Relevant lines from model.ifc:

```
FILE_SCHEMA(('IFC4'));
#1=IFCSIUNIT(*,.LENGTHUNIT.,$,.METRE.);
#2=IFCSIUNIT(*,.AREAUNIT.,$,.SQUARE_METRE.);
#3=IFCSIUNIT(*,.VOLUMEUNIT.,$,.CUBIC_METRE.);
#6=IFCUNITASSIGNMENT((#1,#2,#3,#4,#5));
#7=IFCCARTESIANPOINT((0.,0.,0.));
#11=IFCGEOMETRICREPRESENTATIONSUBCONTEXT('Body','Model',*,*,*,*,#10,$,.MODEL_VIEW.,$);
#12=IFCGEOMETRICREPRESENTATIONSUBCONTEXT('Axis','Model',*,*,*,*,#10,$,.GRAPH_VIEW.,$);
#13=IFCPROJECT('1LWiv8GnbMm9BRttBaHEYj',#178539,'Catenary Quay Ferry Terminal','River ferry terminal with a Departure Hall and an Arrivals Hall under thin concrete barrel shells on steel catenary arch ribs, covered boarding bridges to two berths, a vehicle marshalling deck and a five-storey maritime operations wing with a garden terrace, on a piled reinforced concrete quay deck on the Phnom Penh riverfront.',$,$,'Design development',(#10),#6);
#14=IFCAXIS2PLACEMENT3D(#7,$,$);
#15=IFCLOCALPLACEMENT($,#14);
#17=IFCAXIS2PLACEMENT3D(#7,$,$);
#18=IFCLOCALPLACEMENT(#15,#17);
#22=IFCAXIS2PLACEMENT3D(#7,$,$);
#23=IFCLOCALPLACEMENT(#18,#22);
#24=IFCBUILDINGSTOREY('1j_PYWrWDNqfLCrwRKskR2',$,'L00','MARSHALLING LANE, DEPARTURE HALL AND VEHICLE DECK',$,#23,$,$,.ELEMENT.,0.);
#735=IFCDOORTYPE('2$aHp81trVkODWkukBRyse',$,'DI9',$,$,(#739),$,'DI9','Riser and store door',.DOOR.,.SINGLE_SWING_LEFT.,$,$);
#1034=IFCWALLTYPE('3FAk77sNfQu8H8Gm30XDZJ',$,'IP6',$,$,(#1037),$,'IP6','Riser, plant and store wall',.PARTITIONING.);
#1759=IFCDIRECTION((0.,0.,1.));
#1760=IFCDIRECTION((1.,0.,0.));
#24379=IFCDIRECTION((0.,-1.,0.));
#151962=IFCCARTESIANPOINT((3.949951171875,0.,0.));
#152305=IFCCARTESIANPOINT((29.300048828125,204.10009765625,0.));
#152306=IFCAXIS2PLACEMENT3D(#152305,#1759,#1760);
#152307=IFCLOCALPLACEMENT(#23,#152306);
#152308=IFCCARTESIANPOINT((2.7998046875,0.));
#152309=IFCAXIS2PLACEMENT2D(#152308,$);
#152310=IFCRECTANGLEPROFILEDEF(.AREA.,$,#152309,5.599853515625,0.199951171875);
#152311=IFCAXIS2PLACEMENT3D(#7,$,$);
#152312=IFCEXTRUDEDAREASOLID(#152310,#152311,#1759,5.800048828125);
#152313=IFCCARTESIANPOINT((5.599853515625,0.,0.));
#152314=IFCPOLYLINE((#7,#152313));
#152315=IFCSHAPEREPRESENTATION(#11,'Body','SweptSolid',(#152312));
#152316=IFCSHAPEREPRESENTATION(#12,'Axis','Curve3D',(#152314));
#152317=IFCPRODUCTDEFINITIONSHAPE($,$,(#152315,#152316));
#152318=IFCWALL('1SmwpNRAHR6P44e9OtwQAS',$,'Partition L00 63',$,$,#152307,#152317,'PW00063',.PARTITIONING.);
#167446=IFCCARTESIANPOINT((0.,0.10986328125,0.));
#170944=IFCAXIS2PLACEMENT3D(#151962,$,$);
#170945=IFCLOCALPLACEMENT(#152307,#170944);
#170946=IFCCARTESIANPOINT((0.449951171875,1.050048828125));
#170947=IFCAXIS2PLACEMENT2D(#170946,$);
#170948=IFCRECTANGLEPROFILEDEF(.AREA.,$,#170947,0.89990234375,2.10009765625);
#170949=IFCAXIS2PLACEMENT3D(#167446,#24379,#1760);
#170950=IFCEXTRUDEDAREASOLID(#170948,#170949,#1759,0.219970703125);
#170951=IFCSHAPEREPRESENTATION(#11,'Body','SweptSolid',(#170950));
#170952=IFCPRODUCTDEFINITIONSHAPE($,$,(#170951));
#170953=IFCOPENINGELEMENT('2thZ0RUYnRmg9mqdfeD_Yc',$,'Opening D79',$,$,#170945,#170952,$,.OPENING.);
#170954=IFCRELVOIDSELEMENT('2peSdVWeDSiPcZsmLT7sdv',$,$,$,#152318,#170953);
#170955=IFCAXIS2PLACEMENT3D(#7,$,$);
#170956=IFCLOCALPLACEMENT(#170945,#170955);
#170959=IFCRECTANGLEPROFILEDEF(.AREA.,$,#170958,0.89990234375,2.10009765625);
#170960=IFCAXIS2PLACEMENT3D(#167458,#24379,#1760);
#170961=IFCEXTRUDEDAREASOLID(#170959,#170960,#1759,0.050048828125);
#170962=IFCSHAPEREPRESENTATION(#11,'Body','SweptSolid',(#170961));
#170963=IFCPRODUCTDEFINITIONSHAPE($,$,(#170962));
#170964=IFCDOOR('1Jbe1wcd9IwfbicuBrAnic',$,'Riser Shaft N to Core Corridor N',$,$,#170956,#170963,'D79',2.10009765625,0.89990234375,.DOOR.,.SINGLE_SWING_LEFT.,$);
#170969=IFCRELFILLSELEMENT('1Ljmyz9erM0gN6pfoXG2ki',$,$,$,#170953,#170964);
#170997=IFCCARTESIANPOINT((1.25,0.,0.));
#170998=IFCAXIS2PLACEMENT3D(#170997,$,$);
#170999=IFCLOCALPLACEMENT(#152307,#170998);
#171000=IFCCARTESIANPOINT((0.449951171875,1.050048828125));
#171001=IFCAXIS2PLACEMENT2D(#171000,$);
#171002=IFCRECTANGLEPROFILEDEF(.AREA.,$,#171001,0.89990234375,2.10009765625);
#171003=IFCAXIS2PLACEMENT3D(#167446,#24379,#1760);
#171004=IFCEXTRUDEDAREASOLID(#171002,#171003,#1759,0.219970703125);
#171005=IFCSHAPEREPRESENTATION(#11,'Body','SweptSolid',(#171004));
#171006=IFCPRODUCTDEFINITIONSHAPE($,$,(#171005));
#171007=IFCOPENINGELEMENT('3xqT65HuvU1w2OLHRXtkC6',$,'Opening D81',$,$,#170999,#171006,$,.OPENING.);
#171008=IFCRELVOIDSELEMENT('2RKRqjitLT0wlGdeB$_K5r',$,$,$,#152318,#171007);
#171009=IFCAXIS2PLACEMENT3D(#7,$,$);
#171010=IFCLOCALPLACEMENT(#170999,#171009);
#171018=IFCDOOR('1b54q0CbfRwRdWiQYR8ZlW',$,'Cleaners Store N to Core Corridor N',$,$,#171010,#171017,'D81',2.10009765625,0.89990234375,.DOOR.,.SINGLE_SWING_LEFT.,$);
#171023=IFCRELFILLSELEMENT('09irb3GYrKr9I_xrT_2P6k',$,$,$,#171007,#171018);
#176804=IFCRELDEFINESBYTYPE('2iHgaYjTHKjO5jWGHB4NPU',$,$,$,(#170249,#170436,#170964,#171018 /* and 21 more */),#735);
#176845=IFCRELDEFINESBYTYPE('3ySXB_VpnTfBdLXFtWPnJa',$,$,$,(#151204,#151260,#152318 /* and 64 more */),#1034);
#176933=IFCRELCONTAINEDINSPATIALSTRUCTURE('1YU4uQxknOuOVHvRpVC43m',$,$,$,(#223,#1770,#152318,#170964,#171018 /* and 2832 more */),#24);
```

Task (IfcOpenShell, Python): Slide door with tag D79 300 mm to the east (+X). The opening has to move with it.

```python
import ifcopenshell
import ifcopenshell.api.geometry
import ifcopenshell.util.placement
import ifcopenshell.util.unit

model = ifcopenshell.open("model.ifc")
unit_scale = ifcopenshell.util.unit.calculate_unit_scale(model)

door = model.by_guid("1Jbe1wcd9IwfbicuBrAnic")
opening = door.FillsVoids[0].RelatingOpeningElement
wall = opening.VoidsElements[0].RelatingBuildingElement

wall_matrix = ifcopenshell.util.placement.get_local_placement(wall.ObjectPlacement)
shift = wall_matrix[:3, 0] * 0.3 / unit_scale
before = ifcopenshell.util.placement.get_local_placement(door.ObjectPlacement)[:3, 3].copy()

# The door is placed relative to its opening, so it follows when the opening moves.
matrix = ifcopenshell.util.placement.get_local_placement(opening.ObjectPlacement)
matrix[:3, 3] += shift
ifcopenshell.api.geometry.edit_object_placement(
    model, product=opening, matrix=matrix, is_si=False, should_transform_children=True
)

after = ifcopenshell.util.placement.get_local_placement(door.ObjectPlacement)[:3, 3]
print("door moved by", (after - before).round(3) + 0.0)

model.write("model_edited.ifc")
```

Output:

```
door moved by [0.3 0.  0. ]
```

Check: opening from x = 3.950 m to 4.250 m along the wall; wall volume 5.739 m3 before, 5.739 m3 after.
